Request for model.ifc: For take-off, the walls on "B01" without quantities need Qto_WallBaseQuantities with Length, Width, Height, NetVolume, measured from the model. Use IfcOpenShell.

First a look at what the model holds.

```python
import ifcopenshell
import ifcopenshell.util.element
import ifcopenshell.util.unit

model = ifcopenshell.open("model.ifc")
print(model.schema)
for unit_type in ("LENGTHUNIT", "AREAUNIT", "VOLUMEUNIT"):
    print(unit_type, ifcopenshell.util.unit.calculate_unit_scale(model, unit_type))
storey = next(s for s in model.by_type("IfcBuildingStorey") if s.Name == "B01")
walls = [e for e in ifcopenshell.util.element.get_decomposition(storey) if e.is_a("IfcWall")]
for e in sorted(walls, key=lambda e: e.id()):
    print(e.id(), e.is_a(), e.Name, list(ifcopenshell.util.element.get_psets(e, qtos_only=True)), sep=" | ")
```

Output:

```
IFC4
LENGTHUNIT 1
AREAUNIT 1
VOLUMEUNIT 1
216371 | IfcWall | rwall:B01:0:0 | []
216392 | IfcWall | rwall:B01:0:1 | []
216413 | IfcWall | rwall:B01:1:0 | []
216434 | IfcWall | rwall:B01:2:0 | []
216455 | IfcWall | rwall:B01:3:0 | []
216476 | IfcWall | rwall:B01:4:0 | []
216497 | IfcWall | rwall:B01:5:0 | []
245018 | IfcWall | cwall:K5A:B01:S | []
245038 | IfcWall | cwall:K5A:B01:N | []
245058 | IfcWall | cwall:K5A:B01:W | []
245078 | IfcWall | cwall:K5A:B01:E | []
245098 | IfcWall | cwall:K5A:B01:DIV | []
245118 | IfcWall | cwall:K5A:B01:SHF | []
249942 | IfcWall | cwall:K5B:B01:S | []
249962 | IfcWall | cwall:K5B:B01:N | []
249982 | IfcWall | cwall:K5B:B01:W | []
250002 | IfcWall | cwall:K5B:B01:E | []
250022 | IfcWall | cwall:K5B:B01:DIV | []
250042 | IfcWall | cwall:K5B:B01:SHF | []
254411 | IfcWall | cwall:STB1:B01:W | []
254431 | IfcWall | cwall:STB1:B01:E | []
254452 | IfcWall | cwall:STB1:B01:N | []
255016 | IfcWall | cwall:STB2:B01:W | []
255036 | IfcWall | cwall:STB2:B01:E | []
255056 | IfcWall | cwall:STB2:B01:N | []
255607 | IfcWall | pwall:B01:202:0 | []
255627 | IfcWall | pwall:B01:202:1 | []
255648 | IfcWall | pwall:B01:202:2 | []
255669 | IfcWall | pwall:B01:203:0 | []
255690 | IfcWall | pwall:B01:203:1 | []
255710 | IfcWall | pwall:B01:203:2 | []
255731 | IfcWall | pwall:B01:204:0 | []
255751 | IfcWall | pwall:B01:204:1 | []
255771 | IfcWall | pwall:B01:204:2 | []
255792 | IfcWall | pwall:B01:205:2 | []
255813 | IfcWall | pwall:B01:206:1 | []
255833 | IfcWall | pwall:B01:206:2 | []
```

```python
import ifcopenshell
import ifcopenshell.api.pset
import ifcopenshell.geom
import ifcopenshell.util.element
import ifcopenshell.util.shape
import ifcopenshell.util.unit

model = ifcopenshell.open("model.ifc")
unit_scale = ifcopenshell.util.unit.calculate_unit_scale(model)
volume_scale = ifcopenshell.util.unit.calculate_unit_scale(model, "VOLUMEUNIT")
settings = ifcopenshell.geom.settings()

storey = next(s for s in model.by_type("IfcBuildingStorey") if s.Name == "B01")
walls = [e for e in ifcopenshell.util.element.get_decomposition(storey) if e.is_a("IfcWall")]

for e in sorted(walls, key=lambda e: e.id()):
    if ifcopenshell.util.element.get_psets(e, qtos_only=True, should_inherit=False):
        continue
    # Geometry comes back in metres, in the element's own axes.
    shape = ifcopenshell.geom.create_shape(settings, e)
    values = {
        "Length": ifcopenshell.util.shape.get_x(shape.geometry) / unit_scale,
        "Width": ifcopenshell.util.shape.get_y(shape.geometry) / unit_scale,
        "Height": ifcopenshell.util.shape.get_z(shape.geometry) / unit_scale,
        "NetVolume": ifcopenshell.util.shape.get_volume(shape.geometry) / volume_scale,
    }
    qto = ifcopenshell.api.pset.add_qto(model, product=e, name="Qto_WallBaseQuantities")
    ifcopenshell.api.pset.edit_qto(model, qto=qto, properties=values)
    print(e.id(), {k: round(v, 3) for k, v in values.items()})

model.write("model_rev.ifc")
```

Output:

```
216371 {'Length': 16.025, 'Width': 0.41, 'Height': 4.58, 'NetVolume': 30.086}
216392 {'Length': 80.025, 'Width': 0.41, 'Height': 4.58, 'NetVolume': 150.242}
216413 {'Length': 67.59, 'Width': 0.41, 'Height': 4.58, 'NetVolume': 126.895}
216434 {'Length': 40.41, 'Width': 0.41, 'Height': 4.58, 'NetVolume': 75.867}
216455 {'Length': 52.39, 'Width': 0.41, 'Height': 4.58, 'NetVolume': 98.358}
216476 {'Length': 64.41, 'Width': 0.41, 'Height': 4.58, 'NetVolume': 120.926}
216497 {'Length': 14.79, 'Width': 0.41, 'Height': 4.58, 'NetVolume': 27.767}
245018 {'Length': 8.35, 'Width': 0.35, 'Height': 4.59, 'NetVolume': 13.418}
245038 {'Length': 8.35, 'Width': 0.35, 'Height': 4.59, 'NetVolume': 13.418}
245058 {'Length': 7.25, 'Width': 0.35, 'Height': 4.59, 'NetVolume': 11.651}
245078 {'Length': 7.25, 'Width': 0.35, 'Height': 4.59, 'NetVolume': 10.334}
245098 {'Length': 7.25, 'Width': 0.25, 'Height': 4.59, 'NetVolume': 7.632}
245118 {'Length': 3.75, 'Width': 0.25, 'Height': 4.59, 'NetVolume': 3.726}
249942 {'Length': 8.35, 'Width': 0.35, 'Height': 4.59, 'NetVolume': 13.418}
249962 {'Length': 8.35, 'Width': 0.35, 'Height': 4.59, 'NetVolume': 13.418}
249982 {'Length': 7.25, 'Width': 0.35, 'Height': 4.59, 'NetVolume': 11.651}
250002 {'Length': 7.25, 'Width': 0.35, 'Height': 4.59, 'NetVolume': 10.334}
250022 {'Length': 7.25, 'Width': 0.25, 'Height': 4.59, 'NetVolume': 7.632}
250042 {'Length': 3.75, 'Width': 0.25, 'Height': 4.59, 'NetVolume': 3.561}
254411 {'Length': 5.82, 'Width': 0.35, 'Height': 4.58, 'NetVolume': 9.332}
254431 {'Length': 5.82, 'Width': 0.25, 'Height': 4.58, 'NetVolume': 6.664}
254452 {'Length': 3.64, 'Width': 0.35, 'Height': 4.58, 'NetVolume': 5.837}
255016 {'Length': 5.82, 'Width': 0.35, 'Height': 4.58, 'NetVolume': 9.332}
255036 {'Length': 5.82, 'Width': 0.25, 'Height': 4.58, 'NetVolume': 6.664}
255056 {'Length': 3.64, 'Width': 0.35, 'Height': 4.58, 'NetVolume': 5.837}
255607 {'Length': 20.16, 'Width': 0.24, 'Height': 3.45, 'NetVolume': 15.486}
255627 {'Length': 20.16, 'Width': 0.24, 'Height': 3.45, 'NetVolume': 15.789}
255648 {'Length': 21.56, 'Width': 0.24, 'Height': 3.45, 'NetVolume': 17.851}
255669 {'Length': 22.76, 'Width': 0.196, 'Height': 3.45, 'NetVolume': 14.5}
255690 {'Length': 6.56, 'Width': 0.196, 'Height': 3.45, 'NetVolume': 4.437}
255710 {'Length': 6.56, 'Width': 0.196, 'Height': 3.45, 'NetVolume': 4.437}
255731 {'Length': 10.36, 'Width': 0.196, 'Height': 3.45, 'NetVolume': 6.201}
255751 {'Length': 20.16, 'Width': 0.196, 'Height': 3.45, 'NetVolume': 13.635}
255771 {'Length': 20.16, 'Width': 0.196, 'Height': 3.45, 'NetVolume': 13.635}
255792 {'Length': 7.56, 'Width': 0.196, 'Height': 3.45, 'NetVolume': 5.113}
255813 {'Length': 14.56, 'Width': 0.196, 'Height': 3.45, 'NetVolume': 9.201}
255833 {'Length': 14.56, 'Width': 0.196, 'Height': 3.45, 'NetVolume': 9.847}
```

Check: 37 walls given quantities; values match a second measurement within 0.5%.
